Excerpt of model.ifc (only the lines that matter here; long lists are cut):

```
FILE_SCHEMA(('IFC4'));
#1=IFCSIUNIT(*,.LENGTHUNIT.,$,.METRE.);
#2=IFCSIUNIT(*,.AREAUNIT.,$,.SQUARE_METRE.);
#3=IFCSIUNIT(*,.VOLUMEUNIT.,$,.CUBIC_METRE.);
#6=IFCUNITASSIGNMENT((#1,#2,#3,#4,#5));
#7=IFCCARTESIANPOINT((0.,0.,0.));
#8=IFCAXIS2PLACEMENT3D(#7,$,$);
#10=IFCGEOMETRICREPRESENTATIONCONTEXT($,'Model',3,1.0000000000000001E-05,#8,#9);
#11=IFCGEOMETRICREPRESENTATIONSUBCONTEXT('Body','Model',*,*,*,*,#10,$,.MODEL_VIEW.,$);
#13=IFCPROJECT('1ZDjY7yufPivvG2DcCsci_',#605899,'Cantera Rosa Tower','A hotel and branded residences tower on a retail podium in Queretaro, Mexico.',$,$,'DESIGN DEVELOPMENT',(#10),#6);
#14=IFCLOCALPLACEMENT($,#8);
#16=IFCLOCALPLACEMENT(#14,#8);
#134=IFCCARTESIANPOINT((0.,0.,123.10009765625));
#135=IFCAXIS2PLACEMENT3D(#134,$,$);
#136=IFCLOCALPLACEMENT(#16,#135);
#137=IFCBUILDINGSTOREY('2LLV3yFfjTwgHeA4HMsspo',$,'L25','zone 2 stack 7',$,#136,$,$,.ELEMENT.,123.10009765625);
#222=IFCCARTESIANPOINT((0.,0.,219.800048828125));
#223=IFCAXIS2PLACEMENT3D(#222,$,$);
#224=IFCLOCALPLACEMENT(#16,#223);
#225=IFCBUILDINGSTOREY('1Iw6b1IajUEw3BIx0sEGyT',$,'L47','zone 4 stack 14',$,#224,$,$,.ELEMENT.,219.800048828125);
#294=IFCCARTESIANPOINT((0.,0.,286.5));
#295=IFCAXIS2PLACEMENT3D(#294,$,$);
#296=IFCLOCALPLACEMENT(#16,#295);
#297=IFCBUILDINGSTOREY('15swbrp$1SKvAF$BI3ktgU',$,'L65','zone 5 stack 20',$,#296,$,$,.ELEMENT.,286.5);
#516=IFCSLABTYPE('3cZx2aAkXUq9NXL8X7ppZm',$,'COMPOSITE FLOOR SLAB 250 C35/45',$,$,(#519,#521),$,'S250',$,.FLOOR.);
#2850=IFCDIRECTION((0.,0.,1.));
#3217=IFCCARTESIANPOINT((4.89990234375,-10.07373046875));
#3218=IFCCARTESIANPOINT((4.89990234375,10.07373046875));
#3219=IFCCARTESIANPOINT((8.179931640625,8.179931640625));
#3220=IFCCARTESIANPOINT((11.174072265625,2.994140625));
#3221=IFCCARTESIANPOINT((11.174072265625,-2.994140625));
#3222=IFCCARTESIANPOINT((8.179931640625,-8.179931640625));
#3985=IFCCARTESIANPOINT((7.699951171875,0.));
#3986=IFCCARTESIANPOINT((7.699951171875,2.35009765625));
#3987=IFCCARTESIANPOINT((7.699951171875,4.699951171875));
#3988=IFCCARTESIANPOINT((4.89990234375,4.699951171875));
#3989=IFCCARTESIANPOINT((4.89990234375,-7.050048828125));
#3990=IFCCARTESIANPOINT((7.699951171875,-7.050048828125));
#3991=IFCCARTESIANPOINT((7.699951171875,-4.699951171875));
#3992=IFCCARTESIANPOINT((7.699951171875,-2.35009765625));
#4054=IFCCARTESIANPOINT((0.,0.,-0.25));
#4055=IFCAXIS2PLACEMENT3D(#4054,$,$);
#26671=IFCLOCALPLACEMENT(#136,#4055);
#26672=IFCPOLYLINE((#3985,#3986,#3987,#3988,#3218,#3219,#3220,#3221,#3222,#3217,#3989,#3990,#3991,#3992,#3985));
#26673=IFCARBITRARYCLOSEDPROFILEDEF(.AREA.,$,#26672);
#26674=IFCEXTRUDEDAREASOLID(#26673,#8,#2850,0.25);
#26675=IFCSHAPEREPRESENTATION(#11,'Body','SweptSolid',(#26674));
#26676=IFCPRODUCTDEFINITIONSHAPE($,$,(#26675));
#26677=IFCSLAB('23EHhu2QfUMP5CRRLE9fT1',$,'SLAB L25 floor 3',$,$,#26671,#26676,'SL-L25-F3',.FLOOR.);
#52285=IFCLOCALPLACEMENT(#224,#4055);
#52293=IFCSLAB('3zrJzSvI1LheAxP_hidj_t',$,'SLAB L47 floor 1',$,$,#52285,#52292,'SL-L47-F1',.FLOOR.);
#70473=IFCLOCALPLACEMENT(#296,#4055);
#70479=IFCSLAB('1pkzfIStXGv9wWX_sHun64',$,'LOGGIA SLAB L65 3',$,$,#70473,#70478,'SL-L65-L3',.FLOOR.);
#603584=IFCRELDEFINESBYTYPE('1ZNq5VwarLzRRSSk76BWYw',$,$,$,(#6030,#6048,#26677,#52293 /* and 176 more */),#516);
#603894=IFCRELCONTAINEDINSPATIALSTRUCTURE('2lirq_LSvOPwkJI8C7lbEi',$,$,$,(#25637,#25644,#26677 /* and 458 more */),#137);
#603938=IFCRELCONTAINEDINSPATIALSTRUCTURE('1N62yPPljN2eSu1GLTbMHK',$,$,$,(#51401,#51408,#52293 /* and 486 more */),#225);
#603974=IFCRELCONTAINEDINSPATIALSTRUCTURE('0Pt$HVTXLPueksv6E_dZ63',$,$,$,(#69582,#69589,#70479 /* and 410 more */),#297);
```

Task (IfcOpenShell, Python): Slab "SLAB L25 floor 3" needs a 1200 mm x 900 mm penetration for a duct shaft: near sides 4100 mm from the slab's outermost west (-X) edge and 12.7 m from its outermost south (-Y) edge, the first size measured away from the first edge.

```python
import numpy as np
import ifcopenshell
import ifcopenshell.api.feature
import ifcopenshell.api.geometry
import ifcopenshell.api.root
import ifcopenshell.geom
import ifcopenshell.util.placement
import ifcopenshell.util.representation
import ifcopenshell.util.shape
import ifcopenshell.util.unit

model = ifcopenshell.open("model.ifc")
unit_scale = ifcopenshell.util.unit.calculate_unit_scale(model)
settings = ifcopenshell.geom.settings()


def volume(element):
    """Net volume in cubic metres, openings subtracted."""
    shape = ifcopenshell.geom.create_shape(settings, element)
    return ifcopenshell.util.shape.get_volume(shape.geometry)


slab = model.by_id(26677)
before = volume(slab)

# Extent in the slab's own axes, in metres. The edges named are its -X and -Y sides.
slab_shape = ifcopenshell.geom.create_shape(settings, slab)
vertices = ifcopenshell.util.shape.get_vertices(slab_shape.geometry)
x_min, y_min, bottom = vertices.min(axis=0)
top = vertices[:, 2].max()

opening = ifcopenshell.api.root.create_entity(model, ifc_class="IfcOpeningElement", name="Duct shaft opening", predefined_type="OPENING")
context = ifcopenshell.util.representation.get_context(model, "Model", "Body", "MODEL_VIEW")
width, depth = 1.2, 0.9
outline = [(0.0, 0.0), (width, 0.0), (width, depth), (0.0, depth), (0.0, 0.0)]
# Overshoot both faces by 50 mm so the cut is clean.
shape = ifcopenshell.api.geometry.add_slab_representation(
    model, context=context, depth=top - bottom + 0.1, polyline=outline
)
ifcopenshell.api.geometry.assign_representation(model, product=opening, representation=shape)

matrix = ifcopenshell.util.placement.get_local_placement(slab.ObjectPlacement)
matrix[:, 3] = matrix @ np.append(np.array([x_min + 4.1, y_min + 12.7, bottom - 0.05]) / unit_scale, 1.0)
ifcopenshell.api.geometry.edit_object_placement(model, product=opening, matrix=matrix, is_si=False)
ifcopenshell.api.feature.add_feature(model, feature=opening, element=slab)

after = volume(slab)

print(f"slab volume {before:.3f} -> {after:.3f} m3")

model.write("model-out.ifc")
```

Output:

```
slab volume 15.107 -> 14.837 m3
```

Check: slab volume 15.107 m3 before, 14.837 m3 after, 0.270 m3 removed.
